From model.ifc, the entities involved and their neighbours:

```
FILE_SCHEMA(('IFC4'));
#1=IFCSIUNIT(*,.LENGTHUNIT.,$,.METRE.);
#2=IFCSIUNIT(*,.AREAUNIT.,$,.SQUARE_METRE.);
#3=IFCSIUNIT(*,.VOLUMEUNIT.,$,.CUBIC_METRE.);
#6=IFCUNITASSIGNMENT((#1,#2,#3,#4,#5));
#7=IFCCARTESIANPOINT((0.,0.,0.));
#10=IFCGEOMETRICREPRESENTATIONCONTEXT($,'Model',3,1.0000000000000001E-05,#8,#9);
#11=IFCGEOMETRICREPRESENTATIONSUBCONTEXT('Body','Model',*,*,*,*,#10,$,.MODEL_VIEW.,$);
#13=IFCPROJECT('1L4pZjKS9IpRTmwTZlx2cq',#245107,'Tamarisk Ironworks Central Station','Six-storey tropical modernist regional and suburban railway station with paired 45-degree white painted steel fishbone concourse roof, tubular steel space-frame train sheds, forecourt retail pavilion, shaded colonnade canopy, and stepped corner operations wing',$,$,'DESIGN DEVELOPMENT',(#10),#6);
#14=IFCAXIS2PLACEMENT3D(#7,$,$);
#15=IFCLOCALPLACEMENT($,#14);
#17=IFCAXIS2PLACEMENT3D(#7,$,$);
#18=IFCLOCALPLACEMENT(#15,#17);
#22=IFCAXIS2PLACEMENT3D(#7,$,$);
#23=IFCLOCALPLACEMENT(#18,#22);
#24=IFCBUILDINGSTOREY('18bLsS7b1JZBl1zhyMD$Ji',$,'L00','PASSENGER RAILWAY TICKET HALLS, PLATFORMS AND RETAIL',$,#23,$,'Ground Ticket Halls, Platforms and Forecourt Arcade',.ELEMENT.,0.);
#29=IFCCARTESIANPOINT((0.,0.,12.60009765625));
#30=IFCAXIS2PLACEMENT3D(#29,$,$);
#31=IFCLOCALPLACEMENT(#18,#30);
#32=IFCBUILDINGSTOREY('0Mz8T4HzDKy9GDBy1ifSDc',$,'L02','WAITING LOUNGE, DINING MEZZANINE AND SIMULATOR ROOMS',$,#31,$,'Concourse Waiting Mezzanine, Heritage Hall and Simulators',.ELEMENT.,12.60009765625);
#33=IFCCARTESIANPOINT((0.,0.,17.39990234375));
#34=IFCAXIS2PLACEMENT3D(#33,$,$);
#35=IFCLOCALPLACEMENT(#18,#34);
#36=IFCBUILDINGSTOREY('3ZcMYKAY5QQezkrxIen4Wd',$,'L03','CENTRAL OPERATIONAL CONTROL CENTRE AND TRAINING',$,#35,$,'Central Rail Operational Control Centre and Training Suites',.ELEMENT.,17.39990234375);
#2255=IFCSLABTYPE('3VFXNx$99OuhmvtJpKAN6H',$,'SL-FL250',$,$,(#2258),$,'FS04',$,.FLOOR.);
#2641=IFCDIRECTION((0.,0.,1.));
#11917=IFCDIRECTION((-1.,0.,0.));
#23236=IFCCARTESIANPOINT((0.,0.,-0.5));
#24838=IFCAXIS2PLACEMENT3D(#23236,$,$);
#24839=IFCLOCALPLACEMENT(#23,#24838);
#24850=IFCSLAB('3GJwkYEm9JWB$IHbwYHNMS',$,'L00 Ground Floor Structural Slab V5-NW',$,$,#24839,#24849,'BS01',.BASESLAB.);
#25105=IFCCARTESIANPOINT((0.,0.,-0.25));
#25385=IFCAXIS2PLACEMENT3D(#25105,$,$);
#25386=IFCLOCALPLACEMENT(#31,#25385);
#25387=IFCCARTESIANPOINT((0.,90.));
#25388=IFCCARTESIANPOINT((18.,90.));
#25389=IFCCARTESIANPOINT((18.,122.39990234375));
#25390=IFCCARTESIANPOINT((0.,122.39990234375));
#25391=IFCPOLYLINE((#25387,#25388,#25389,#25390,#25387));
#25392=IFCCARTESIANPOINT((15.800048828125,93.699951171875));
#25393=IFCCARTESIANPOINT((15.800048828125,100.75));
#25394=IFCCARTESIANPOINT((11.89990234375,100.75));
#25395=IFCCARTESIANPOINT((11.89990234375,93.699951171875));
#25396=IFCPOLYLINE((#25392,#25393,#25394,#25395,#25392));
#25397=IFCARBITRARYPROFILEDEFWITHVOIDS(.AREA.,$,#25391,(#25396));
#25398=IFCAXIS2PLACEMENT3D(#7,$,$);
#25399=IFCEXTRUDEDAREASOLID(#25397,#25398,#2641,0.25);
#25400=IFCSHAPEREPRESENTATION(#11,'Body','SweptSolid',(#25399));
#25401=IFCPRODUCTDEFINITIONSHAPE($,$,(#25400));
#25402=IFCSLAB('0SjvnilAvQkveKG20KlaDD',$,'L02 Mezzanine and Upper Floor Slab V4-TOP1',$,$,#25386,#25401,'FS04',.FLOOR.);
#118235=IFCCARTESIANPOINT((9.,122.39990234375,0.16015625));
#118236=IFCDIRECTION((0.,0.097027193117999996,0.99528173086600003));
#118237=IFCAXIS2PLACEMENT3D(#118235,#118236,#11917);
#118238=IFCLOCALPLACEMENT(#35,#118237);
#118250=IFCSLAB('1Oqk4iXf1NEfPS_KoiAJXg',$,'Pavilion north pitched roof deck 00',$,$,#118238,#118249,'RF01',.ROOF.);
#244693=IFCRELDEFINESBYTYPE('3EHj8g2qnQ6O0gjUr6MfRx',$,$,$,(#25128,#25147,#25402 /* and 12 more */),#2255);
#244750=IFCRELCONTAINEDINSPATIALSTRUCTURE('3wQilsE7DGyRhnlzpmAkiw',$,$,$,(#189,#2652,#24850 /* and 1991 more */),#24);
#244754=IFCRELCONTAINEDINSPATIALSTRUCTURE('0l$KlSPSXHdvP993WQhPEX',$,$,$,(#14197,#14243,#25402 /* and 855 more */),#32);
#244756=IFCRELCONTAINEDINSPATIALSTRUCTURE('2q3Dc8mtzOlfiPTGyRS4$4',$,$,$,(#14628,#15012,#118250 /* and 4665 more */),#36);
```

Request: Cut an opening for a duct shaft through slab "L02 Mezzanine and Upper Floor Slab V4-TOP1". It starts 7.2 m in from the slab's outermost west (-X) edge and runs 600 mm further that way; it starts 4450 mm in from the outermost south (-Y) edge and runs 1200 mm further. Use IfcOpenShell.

```python
import numpy as np
import ifcopenshell
import ifcopenshell.api.feature
import ifcopenshell.api.geometry
import ifcopenshell.api.root
import ifcopenshell.geom
import ifcopenshell.util.placement
import ifcopenshell.util.representation
import ifcopenshell.util.shape
import ifcopenshell.util.unit

model = ifcopenshell.open("model.ifc")
unit_scale = ifcopenshell.util.unit.calculate_unit_scale(model)
settings = ifcopenshell.geom.settings()


def volume(element):
    """Net volume in cubic metres, openings subtracted."""
    shape = ifcopenshell.geom.create_shape(settings, element)
    return ifcopenshell.util.shape.get_volume(shape.geometry)


slab = model.by_guid("0SjvnilAvQkveKG20KlaDD")
before = volume(slab)

# Extent in the slab's own axes, in metres. The edges named are its -X and -Y sides.
slab_shape = ifcopenshell.geom.create_shape(settings, slab)
vertices = ifcopenshell.util.shape.get_vertices(slab_shape.geometry)
x_min, y_min, bottom = vertices.min(axis=0)
top = vertices[:, 2].max()

opening = ifcopenshell.api.root.create_entity(model, ifc_class="IfcOpeningElement", name="Duct shaft opening", predefined_type="OPENING")
context = ifcopenshell.util.representation.get_context(model, "Model", "Body", "MODEL_VIEW")
width, depth = 0.6, 1.2
outline = [(0.0, 0.0), (width, 0.0), (width, depth), (0.0, depth), (0.0, 0.0)]
# Overshoot both faces by 50 mm so the cut is clean.
shape = ifcopenshell.api.geometry.add_slab_representation(
    model, context=context, depth=top - bottom + 0.1, polyline=outline
)
ifcopenshell.api.geometry.assign_representation(model, product=opening, representation=shape)

matrix = ifcopenshell.util.placement.get_local_placement(slab.ObjectPlacement)
matrix[:, 3] = matrix @ np.append(np.array([x_min + 7.2, y_min + 4.45, bottom - 0.05]) / unit_scale, 1.0)
ifcopenshell.api.geometry.edit_object_placement(model, product=opening, matrix=matrix, is_si=False)
ifcopenshell.api.feature.add_feature(model, feature=opening, element=slab)

after = volume(slab)

print(f"slab volume {before:.3f} -> {after:.3f} m3")

model.write("model_rev.ifc")
```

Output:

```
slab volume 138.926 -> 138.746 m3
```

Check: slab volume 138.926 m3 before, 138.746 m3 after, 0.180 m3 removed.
